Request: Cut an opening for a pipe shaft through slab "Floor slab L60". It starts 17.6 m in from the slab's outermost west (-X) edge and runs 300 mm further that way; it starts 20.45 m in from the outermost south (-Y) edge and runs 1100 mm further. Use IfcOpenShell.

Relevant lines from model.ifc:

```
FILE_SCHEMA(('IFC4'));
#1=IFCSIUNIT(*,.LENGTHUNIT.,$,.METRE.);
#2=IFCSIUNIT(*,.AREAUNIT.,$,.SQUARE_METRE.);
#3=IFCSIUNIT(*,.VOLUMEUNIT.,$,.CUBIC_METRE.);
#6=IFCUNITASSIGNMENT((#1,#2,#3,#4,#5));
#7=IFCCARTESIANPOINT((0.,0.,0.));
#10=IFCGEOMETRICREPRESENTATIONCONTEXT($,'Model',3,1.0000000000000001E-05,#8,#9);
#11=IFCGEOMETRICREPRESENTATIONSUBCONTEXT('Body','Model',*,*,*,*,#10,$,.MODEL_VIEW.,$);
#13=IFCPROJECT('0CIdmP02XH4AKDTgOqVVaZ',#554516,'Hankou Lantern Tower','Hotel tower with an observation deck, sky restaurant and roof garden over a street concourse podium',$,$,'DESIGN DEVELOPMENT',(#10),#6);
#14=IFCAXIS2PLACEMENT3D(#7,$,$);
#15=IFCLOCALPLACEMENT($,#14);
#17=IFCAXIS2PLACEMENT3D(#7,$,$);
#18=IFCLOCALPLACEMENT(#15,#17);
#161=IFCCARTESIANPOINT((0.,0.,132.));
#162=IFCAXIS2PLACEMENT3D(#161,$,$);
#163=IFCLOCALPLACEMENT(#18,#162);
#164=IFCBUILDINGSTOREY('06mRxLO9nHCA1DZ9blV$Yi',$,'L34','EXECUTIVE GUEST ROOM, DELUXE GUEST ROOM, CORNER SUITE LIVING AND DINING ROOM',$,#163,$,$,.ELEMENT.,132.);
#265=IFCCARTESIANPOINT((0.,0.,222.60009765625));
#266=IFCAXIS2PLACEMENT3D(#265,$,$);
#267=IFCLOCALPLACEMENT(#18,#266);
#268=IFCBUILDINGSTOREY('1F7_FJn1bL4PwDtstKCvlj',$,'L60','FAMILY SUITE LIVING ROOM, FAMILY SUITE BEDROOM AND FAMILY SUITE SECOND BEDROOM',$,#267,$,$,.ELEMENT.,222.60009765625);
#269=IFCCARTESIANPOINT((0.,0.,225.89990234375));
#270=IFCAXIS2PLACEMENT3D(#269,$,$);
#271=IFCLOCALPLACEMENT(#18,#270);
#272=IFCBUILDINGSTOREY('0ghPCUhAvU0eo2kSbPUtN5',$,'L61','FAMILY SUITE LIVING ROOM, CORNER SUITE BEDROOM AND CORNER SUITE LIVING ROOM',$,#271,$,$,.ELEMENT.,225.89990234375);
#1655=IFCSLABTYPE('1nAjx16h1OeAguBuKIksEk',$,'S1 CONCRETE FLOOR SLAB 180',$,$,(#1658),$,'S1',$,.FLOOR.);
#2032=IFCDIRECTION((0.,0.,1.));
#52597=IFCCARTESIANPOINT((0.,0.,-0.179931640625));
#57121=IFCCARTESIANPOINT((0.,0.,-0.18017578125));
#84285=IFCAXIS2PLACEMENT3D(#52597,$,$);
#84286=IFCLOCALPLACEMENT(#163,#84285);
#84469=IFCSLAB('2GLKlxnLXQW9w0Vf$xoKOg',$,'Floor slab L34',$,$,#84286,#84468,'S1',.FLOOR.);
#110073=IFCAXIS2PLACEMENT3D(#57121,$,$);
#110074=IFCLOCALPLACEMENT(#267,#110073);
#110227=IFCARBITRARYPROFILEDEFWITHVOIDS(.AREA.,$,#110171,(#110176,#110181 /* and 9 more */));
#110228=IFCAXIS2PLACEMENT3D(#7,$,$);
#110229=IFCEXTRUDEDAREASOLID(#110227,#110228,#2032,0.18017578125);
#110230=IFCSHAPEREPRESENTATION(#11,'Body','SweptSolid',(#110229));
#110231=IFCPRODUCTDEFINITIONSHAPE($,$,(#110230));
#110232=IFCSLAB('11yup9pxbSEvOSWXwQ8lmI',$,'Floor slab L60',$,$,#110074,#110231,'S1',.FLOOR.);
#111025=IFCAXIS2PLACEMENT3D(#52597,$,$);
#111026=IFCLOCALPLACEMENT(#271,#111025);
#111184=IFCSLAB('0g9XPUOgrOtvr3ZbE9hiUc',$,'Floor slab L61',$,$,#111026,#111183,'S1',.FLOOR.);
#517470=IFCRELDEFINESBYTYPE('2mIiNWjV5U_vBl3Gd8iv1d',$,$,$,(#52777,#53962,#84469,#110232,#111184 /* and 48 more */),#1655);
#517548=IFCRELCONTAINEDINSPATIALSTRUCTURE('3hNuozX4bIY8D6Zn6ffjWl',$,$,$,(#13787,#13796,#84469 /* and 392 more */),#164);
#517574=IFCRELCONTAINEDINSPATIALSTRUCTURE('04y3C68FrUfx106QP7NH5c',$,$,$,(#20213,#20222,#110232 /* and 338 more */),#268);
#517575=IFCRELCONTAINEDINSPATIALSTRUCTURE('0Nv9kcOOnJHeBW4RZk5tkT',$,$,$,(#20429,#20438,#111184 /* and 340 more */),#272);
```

```python
import numpy as np
import ifcopenshell
import ifcopenshell.api.feature
import ifcopenshell.api.geometry
import ifcopenshell.api.root
import ifcopenshell.geom
import ifcopenshell.util.placement
import ifcopenshell.util.representation
import ifcopenshell.util.shape
import ifcopenshell.util.unit

model = ifcopenshell.open("model.ifc")
unit_scale = ifcopenshell.util.unit.calculate_unit_scale(model)
settings = ifcopenshell.geom.settings()


def volume(element):
    """Net volume in cubic metres, openings subtracted."""
    shape = ifcopenshell.geom.create_shape(settings, element)
    return ifcopenshell.util.shape.get_volume(shape.geometry)


slab = model.by_guid("11yup9pxbSEvOSWXwQ8lmI")
before = volume(slab)

# Extent in the slab's own axes, in metres. The edges named are its -X and -Y sides.
slab_shape = ifcopenshell.geom.create_shape(settings, slab)
vertices = ifcopenshell.util.shape.get_vertices(slab_shape.geometry)
x_min, y_min, bottom = vertices.min(axis=0)
top = vertices[:, 2].max()

opening = ifcopenshell.api.root.create_entity(model, ifc_class="IfcOpeningElement", name="Pipe shaft opening", predefined_type="OPENING")
context = ifcopenshell.util.representation.get_context(model, "Model", "Body", "MODEL_VIEW")
width, depth = 0.3, 1.1
outline = [(0.0, 0.0), (width, 0.0), (width, depth), (0.0, depth), (0.0, 0.0)]
# Overshoot both faces by 50 mm so the cut is clean.
shape = ifcopenshell.api.geometry.add_slab_representation(
    model, context=context, depth=top - bottom + 0.1, polyline=outline
)
ifcopenshell.api.geometry.assign_representation(model, product=opening, representation=shape)

matrix = ifcopenshell.util.placement.get_local_placement(slab.ObjectPlacement)
matrix[:, 3] = matrix @ np.append(np.array([x_min + 17.6, y_min + 20.45, bottom - 0.05]) / unit_scale, 1.0)
ifcopenshell.api.geometry.edit_object_placement(model, product=opening, matrix=matrix, is_si=False)
ifcopenshell.api.feature.add_feature(model, feature=opening, element=slab)

after = volume(slab)

print(f"slab volume {before:.3f} -> {after:.3f} m3")

model.write("model_rev.ifc")
```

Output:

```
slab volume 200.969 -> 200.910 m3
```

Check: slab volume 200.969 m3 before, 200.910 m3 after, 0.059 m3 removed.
